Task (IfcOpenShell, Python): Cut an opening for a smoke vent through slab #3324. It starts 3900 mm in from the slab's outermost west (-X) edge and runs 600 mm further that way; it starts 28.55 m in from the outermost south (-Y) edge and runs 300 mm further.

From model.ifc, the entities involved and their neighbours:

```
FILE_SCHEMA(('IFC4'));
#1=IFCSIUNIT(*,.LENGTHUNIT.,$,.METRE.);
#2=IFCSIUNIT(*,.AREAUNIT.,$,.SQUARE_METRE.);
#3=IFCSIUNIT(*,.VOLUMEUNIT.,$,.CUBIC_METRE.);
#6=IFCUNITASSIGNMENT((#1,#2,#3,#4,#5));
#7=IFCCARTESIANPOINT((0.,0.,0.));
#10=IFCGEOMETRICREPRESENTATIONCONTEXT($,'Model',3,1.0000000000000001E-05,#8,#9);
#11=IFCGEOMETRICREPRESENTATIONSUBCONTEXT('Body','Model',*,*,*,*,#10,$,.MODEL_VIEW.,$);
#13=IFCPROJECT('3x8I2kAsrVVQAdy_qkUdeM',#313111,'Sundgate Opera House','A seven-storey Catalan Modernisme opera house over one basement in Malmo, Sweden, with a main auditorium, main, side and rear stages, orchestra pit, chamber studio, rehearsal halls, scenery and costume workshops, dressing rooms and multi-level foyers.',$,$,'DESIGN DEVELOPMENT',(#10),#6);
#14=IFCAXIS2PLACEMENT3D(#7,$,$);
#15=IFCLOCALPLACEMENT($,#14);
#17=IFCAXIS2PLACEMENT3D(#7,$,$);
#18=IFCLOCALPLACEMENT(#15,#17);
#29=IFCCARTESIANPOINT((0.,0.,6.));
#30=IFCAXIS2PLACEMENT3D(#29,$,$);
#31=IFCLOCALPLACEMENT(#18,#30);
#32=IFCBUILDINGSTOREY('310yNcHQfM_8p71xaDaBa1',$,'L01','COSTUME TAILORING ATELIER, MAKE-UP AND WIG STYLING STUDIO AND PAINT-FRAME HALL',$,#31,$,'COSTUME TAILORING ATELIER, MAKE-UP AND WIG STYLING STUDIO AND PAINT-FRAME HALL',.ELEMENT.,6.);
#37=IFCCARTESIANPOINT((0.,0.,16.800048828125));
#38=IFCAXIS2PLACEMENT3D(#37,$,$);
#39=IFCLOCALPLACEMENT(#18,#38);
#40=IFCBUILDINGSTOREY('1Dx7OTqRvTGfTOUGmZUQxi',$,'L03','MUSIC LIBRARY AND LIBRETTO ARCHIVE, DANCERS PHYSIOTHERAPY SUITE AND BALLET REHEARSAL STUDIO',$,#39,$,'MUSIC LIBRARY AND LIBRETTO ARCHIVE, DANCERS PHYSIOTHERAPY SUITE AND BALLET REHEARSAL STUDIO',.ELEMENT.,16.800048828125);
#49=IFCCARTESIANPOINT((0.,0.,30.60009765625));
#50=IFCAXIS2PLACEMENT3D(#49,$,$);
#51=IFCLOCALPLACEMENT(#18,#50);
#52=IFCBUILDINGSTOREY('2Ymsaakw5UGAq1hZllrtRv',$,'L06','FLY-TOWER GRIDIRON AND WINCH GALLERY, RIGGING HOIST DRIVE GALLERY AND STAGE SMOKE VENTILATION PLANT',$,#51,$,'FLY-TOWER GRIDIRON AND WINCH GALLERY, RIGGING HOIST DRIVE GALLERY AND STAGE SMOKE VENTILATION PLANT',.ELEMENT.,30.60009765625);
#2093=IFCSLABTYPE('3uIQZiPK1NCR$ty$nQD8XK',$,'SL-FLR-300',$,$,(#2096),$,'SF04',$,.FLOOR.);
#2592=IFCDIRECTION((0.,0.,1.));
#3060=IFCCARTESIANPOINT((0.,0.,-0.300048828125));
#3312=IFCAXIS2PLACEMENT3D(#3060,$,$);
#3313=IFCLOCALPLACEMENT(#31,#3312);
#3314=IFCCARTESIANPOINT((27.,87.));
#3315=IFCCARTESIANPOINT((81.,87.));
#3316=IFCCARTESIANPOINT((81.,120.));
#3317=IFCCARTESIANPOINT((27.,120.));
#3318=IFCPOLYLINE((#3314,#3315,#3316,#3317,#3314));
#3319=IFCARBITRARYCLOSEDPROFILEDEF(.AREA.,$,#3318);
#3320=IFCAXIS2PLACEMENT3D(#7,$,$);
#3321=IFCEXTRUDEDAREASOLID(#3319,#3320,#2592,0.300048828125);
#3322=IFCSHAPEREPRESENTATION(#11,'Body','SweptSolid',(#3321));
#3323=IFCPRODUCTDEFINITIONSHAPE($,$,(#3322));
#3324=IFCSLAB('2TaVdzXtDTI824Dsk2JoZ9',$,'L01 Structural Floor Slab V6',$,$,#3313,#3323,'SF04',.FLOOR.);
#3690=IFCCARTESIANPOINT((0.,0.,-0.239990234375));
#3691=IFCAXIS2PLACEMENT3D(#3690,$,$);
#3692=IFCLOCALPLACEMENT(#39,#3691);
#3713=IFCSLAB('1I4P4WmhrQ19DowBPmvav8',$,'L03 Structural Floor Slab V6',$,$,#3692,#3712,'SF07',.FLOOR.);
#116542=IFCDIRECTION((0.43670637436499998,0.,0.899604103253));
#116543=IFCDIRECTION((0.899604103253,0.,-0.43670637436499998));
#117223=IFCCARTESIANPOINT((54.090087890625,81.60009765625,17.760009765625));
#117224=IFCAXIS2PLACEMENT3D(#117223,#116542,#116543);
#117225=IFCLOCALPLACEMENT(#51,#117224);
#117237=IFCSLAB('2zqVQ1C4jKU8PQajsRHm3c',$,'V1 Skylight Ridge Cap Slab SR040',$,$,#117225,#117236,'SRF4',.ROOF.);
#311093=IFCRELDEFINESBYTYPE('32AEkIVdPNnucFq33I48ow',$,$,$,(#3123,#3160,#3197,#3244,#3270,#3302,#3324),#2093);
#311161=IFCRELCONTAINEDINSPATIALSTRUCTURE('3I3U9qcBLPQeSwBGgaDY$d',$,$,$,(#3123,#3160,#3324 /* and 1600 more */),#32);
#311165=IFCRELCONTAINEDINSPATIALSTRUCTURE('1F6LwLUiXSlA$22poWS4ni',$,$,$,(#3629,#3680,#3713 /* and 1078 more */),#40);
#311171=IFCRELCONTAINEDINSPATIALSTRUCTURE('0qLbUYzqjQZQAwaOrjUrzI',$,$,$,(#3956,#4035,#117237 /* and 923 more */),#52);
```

```python
import numpy as np
import ifcopenshell
import ifcopenshell.api.feature
import ifcopenshell.api.geometry
import ifcopenshell.api.root
import ifcopenshell.geom
import ifcopenshell.util.placement
import ifcopenshell.util.representation
import ifcopenshell.util.shape
import ifcopenshell.util.unit

model = ifcopenshell.open("model.ifc")
unit_scale = ifcopenshell.util.unit.calculate_unit_scale(model)
settings = ifcopenshell.geom.settings()


def volume(element):
    """Net volume in cubic metres, openings subtracted."""
    shape = ifcopenshell.geom.create_shape(settings, element)
    return ifcopenshell.util.shape.get_volume(shape.geometry)


slab = model.by_guid("2TaVdzXtDTI824Dsk2JoZ9")
before = volume(slab)

# Extent in the slab's own axes, in metres. The edges named are its -X and -Y sides.
slab_shape = ifcopenshell.geom.create_shape(settings, slab)
vertices = ifcopenshell.util.shape.get_vertices(slab_shape.geometry)
x_min, y_min, bottom = vertices.min(axis=0)
top = vertices[:, 2].max()

opening = ifcopenshell.api.root.create_entity(model, ifc_class="IfcOpeningElement", name="Smoke vent opening", predefined_type="OPENING")
context = ifcopenshell.util.representation.get_context(model, "Model", "Body", "MODEL_VIEW")
width, depth = 0.6, 0.3
outline = [(0.0, 0.0), (width, 0.0), (width, depth), (0.0, depth), (0.0, 0.0)]
# Overshoot both faces by 50 mm so the cut is clean.
shape = ifcopenshell.api.geometry.add_slab_representation(
    model, context=context, depth=top - bottom + 0.1, polyline=outline
)
ifcopenshell.api.geometry.assign_representation(model, product=opening, representation=shape)

matrix = ifcopenshell.util.placement.get_local_placement(slab.ObjectPlacement)
matrix[:, 3] = matrix @ np.append(np.array([x_min + 3.9, y_min + 28.55, bottom - 0.05]) / unit_scale, 1.0)
ifcopenshell.api.geometry.edit_object_placement(model, product=opening, matrix=matrix, is_si=False)
ifcopenshell.api.feature.add_feature(model, feature=opening, element=slab)

after = volume(slab)

print(f"slab volume {before:.3f} -> {after:.3f} m3")

model.write("model-out.ifc")
```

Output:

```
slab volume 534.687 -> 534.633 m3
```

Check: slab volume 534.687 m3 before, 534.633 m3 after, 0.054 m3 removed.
